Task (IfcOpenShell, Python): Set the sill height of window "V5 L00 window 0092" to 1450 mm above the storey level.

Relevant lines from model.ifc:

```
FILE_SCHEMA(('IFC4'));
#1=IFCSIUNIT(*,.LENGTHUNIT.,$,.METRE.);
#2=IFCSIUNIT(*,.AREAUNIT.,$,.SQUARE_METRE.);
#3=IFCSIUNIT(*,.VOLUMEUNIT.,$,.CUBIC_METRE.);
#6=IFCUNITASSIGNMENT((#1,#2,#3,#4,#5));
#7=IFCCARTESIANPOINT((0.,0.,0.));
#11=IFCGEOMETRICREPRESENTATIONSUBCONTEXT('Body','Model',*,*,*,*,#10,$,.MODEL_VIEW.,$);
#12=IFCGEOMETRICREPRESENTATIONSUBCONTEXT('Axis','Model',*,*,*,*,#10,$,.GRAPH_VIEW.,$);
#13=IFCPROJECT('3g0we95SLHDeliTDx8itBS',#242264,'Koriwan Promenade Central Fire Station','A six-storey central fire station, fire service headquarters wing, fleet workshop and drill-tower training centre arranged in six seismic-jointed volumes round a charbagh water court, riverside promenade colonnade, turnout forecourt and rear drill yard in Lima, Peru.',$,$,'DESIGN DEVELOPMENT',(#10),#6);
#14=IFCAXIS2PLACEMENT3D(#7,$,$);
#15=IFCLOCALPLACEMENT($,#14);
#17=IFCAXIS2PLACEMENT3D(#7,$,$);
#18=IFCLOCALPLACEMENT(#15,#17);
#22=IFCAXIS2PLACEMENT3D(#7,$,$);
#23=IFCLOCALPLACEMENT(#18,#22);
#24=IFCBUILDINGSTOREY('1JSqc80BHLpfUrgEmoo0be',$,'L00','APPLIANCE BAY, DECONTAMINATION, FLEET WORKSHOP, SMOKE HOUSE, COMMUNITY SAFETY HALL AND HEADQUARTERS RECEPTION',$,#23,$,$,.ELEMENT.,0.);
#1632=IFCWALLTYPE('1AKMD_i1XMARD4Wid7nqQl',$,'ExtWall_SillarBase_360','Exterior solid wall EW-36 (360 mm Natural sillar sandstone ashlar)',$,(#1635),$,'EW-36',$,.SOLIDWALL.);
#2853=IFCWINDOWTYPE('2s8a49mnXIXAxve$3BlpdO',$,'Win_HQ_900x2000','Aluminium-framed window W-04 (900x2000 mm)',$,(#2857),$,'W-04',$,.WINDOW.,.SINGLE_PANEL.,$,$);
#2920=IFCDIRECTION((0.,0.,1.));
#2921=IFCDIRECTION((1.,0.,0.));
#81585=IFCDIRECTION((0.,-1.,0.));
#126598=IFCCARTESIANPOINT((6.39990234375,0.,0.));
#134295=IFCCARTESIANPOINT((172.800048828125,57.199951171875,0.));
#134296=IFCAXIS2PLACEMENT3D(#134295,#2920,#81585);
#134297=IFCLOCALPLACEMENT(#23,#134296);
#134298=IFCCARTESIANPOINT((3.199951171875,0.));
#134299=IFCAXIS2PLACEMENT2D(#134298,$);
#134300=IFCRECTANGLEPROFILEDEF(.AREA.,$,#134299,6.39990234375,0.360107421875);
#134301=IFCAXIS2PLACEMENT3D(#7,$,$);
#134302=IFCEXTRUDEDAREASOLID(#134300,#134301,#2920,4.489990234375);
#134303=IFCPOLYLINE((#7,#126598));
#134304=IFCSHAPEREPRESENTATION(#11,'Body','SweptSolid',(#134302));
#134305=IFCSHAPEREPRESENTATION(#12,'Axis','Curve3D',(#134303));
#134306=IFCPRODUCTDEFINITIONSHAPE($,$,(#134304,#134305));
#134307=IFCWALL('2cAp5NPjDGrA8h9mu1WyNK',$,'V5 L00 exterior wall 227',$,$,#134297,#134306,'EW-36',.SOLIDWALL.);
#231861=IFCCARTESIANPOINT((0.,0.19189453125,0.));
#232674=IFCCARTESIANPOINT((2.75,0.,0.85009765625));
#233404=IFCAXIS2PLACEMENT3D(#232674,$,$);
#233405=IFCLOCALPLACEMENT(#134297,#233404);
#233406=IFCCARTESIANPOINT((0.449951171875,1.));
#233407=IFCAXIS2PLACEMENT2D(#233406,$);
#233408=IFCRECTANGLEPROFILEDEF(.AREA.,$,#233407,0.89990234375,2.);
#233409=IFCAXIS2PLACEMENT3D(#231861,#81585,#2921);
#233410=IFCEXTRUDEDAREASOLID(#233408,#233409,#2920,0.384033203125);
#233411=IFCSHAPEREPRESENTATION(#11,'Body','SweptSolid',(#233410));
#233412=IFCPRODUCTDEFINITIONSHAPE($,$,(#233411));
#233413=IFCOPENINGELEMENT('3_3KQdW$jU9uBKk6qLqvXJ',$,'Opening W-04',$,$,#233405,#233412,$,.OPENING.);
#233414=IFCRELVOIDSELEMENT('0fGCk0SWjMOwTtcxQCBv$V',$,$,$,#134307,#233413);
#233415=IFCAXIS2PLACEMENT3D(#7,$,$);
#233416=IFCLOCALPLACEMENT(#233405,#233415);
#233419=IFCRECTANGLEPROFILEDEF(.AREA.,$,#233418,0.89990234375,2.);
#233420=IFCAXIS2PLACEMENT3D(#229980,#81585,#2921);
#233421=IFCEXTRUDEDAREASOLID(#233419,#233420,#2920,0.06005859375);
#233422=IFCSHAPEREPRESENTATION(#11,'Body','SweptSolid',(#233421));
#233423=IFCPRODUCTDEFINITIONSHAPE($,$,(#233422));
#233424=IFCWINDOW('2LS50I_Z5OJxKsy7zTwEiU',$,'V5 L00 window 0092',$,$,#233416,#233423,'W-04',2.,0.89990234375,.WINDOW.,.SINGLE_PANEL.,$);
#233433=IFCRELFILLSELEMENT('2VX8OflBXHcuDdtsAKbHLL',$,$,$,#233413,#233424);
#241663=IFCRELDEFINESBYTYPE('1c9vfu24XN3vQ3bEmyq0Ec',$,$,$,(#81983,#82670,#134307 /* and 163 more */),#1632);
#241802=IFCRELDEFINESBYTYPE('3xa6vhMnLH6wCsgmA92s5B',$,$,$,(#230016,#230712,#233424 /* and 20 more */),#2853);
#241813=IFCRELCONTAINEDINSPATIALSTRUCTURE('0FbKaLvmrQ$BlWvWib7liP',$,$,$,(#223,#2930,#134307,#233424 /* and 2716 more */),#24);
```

```python
import numpy as np
import ifcopenshell
import ifcopenshell.api.geometry
import ifcopenshell.geom
import ifcopenshell.util.element
import ifcopenshell.util.placement
import ifcopenshell.util.shape
import ifcopenshell.util.unit

model = ifcopenshell.open("model.ifc")
unit_scale = ifcopenshell.util.unit.calculate_unit_scale(model)

window = model.by_guid("2LS50I_Z5OJxKsy7zTwEiU")
opening = window.FillsVoids[0].RelatingOpeningElement
storey = ifcopenshell.util.element.get_container(window, ifc_class="IfcBuildingStorey")
level = ifcopenshell.util.placement.get_local_placement(storey.ObjectPlacement)[2, 3]

# The opening's origin need not be at the sill, so measure its lowest point.
shape = ifcopenshell.geom.create_shape(ifcopenshell.geom.settings(), opening)
bottom = ifcopenshell.util.shape.get_shape_bottom_elevation(shape, shape.geometry) / unit_scale
dz = level + 1.45 - bottom

shift = np.array([0.0, 0.0, dz])
# The window is placed relative to its opening, so it follows when the opening moves.
matrix = ifcopenshell.util.placement.get_local_placement(opening.ObjectPlacement)
matrix[:3, 3] += shift
ifcopenshell.api.geometry.edit_object_placement(
    model, product=opening, matrix=matrix, is_si=False, should_transform_children=True
)

print(f"moved by {dz * unit_scale:+.3f} m")

model.write("model_edited.ifc")
```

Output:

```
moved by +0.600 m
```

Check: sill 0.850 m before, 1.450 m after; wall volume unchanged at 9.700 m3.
